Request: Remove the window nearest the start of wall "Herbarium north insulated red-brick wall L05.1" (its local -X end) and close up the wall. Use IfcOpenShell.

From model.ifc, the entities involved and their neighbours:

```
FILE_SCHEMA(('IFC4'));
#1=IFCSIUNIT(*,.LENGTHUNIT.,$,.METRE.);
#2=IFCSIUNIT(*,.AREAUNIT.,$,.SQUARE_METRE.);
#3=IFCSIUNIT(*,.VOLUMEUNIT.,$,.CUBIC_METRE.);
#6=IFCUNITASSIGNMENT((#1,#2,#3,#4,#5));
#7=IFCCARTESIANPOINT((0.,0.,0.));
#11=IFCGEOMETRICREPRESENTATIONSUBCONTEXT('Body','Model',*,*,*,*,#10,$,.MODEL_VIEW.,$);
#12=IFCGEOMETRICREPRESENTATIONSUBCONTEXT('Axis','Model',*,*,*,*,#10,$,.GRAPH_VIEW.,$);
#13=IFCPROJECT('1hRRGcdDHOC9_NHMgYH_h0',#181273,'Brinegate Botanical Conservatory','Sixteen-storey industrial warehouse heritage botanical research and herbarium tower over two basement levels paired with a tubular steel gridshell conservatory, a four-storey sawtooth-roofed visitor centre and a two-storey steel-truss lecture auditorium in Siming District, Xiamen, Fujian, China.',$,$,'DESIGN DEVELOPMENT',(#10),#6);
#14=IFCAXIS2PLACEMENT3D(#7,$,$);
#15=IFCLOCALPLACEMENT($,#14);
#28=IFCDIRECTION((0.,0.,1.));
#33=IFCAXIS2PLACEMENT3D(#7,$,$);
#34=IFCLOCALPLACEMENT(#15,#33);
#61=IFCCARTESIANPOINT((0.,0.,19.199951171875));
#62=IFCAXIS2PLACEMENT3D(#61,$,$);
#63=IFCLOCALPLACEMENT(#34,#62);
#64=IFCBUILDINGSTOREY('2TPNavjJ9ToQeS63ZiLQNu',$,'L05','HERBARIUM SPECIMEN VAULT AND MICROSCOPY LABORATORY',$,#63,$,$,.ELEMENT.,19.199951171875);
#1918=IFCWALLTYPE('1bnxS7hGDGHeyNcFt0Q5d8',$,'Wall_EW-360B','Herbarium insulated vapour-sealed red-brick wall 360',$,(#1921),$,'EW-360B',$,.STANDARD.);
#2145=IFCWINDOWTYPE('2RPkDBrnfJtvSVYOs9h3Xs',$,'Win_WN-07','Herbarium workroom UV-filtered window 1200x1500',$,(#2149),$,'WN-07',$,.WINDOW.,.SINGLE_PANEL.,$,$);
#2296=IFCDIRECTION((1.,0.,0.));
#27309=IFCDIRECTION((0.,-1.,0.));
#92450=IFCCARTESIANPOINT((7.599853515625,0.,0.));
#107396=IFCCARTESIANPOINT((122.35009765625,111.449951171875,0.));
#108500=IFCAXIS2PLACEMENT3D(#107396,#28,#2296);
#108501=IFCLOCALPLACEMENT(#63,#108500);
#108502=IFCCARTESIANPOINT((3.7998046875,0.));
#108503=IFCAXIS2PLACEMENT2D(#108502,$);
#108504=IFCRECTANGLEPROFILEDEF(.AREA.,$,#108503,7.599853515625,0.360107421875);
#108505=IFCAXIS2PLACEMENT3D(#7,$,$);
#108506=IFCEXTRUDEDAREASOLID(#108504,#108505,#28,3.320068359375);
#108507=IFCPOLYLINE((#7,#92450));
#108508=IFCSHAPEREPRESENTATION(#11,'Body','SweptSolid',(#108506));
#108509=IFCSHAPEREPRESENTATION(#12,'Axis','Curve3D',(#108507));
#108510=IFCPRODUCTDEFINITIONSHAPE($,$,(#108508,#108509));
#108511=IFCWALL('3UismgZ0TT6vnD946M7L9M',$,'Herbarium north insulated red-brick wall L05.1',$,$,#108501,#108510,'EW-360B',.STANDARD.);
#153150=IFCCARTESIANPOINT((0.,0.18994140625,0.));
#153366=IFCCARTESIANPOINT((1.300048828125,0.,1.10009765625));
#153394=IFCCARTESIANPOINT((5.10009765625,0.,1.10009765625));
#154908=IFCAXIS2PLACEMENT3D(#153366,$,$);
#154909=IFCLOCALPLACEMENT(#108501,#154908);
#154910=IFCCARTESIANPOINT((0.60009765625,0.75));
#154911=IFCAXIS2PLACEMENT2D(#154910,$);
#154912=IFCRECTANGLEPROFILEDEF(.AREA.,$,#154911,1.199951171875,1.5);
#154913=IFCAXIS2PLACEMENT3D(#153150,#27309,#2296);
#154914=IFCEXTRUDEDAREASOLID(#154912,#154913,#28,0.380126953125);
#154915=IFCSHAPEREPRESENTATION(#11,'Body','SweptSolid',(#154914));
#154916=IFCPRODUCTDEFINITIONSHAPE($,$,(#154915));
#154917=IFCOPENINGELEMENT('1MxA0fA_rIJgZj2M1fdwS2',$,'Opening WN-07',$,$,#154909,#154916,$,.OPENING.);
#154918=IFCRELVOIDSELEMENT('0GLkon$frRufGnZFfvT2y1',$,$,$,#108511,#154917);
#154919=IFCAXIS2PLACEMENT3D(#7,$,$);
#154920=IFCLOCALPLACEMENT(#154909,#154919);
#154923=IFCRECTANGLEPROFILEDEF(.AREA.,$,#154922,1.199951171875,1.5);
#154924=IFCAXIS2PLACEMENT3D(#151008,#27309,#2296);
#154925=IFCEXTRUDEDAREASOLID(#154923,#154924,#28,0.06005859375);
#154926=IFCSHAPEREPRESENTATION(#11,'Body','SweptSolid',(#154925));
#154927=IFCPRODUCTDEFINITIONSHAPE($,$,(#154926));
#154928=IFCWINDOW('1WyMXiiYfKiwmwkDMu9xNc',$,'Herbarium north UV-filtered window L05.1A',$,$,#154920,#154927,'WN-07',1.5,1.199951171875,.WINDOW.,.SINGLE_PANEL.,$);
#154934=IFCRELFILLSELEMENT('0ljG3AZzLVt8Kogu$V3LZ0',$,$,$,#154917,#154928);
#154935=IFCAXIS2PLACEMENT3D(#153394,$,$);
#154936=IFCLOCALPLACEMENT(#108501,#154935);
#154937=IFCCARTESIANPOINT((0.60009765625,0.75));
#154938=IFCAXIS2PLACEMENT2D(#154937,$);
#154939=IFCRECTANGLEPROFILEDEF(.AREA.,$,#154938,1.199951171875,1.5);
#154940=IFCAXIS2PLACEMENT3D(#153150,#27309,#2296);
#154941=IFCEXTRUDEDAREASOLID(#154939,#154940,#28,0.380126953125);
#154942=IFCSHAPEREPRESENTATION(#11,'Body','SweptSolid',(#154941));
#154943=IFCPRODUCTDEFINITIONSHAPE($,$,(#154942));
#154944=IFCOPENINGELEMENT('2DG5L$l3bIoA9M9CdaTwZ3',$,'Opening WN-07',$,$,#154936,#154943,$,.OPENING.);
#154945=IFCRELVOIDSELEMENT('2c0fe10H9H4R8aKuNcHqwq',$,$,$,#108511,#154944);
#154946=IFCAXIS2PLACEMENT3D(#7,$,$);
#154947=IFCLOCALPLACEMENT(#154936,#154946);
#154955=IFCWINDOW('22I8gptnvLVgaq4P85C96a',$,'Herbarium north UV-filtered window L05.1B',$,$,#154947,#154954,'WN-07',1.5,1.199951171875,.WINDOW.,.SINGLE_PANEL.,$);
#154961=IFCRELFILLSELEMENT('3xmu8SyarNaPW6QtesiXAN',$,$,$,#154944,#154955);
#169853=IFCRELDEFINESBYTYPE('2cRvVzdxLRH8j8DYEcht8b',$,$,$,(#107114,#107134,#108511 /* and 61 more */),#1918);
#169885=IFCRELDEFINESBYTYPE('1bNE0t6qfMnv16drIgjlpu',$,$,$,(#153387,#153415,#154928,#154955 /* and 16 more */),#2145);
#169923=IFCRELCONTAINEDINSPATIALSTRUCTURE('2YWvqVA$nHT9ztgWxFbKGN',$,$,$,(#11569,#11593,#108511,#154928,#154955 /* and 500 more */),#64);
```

```python
import ifcopenshell
import ifcopenshell.api.feature
import ifcopenshell.api.root
import ifcopenshell.geom
import ifcopenshell.util.shape

model = ifcopenshell.open("model.ifc")
settings = ifcopenshell.geom.settings()


def volume(element):
    """Net volume in cubic metres, openings subtracted."""
    shape = ifcopenshell.geom.create_shape(settings, element)
    return ifcopenshell.util.shape.get_volume(shape.geometry)


window = model.by_guid("1WyMXiiYfKiwmwkDMu9xNc")
opening = window.FillsVoids[0].RelatingOpeningElement
wall = opening.VoidsElements[0].RelatingBuildingElement
before = volume(wall)

ifcopenshell.api.root.remove_product(model, product=window)
ifcopenshell.api.feature.remove_feature(model, feature=opening)

after = volume(wall)

print(f"wall volume {before:.3f} -> {after:.3f} m3")

model.write("model-out.ifc")
```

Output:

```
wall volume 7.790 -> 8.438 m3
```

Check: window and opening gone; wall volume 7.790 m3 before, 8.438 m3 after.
